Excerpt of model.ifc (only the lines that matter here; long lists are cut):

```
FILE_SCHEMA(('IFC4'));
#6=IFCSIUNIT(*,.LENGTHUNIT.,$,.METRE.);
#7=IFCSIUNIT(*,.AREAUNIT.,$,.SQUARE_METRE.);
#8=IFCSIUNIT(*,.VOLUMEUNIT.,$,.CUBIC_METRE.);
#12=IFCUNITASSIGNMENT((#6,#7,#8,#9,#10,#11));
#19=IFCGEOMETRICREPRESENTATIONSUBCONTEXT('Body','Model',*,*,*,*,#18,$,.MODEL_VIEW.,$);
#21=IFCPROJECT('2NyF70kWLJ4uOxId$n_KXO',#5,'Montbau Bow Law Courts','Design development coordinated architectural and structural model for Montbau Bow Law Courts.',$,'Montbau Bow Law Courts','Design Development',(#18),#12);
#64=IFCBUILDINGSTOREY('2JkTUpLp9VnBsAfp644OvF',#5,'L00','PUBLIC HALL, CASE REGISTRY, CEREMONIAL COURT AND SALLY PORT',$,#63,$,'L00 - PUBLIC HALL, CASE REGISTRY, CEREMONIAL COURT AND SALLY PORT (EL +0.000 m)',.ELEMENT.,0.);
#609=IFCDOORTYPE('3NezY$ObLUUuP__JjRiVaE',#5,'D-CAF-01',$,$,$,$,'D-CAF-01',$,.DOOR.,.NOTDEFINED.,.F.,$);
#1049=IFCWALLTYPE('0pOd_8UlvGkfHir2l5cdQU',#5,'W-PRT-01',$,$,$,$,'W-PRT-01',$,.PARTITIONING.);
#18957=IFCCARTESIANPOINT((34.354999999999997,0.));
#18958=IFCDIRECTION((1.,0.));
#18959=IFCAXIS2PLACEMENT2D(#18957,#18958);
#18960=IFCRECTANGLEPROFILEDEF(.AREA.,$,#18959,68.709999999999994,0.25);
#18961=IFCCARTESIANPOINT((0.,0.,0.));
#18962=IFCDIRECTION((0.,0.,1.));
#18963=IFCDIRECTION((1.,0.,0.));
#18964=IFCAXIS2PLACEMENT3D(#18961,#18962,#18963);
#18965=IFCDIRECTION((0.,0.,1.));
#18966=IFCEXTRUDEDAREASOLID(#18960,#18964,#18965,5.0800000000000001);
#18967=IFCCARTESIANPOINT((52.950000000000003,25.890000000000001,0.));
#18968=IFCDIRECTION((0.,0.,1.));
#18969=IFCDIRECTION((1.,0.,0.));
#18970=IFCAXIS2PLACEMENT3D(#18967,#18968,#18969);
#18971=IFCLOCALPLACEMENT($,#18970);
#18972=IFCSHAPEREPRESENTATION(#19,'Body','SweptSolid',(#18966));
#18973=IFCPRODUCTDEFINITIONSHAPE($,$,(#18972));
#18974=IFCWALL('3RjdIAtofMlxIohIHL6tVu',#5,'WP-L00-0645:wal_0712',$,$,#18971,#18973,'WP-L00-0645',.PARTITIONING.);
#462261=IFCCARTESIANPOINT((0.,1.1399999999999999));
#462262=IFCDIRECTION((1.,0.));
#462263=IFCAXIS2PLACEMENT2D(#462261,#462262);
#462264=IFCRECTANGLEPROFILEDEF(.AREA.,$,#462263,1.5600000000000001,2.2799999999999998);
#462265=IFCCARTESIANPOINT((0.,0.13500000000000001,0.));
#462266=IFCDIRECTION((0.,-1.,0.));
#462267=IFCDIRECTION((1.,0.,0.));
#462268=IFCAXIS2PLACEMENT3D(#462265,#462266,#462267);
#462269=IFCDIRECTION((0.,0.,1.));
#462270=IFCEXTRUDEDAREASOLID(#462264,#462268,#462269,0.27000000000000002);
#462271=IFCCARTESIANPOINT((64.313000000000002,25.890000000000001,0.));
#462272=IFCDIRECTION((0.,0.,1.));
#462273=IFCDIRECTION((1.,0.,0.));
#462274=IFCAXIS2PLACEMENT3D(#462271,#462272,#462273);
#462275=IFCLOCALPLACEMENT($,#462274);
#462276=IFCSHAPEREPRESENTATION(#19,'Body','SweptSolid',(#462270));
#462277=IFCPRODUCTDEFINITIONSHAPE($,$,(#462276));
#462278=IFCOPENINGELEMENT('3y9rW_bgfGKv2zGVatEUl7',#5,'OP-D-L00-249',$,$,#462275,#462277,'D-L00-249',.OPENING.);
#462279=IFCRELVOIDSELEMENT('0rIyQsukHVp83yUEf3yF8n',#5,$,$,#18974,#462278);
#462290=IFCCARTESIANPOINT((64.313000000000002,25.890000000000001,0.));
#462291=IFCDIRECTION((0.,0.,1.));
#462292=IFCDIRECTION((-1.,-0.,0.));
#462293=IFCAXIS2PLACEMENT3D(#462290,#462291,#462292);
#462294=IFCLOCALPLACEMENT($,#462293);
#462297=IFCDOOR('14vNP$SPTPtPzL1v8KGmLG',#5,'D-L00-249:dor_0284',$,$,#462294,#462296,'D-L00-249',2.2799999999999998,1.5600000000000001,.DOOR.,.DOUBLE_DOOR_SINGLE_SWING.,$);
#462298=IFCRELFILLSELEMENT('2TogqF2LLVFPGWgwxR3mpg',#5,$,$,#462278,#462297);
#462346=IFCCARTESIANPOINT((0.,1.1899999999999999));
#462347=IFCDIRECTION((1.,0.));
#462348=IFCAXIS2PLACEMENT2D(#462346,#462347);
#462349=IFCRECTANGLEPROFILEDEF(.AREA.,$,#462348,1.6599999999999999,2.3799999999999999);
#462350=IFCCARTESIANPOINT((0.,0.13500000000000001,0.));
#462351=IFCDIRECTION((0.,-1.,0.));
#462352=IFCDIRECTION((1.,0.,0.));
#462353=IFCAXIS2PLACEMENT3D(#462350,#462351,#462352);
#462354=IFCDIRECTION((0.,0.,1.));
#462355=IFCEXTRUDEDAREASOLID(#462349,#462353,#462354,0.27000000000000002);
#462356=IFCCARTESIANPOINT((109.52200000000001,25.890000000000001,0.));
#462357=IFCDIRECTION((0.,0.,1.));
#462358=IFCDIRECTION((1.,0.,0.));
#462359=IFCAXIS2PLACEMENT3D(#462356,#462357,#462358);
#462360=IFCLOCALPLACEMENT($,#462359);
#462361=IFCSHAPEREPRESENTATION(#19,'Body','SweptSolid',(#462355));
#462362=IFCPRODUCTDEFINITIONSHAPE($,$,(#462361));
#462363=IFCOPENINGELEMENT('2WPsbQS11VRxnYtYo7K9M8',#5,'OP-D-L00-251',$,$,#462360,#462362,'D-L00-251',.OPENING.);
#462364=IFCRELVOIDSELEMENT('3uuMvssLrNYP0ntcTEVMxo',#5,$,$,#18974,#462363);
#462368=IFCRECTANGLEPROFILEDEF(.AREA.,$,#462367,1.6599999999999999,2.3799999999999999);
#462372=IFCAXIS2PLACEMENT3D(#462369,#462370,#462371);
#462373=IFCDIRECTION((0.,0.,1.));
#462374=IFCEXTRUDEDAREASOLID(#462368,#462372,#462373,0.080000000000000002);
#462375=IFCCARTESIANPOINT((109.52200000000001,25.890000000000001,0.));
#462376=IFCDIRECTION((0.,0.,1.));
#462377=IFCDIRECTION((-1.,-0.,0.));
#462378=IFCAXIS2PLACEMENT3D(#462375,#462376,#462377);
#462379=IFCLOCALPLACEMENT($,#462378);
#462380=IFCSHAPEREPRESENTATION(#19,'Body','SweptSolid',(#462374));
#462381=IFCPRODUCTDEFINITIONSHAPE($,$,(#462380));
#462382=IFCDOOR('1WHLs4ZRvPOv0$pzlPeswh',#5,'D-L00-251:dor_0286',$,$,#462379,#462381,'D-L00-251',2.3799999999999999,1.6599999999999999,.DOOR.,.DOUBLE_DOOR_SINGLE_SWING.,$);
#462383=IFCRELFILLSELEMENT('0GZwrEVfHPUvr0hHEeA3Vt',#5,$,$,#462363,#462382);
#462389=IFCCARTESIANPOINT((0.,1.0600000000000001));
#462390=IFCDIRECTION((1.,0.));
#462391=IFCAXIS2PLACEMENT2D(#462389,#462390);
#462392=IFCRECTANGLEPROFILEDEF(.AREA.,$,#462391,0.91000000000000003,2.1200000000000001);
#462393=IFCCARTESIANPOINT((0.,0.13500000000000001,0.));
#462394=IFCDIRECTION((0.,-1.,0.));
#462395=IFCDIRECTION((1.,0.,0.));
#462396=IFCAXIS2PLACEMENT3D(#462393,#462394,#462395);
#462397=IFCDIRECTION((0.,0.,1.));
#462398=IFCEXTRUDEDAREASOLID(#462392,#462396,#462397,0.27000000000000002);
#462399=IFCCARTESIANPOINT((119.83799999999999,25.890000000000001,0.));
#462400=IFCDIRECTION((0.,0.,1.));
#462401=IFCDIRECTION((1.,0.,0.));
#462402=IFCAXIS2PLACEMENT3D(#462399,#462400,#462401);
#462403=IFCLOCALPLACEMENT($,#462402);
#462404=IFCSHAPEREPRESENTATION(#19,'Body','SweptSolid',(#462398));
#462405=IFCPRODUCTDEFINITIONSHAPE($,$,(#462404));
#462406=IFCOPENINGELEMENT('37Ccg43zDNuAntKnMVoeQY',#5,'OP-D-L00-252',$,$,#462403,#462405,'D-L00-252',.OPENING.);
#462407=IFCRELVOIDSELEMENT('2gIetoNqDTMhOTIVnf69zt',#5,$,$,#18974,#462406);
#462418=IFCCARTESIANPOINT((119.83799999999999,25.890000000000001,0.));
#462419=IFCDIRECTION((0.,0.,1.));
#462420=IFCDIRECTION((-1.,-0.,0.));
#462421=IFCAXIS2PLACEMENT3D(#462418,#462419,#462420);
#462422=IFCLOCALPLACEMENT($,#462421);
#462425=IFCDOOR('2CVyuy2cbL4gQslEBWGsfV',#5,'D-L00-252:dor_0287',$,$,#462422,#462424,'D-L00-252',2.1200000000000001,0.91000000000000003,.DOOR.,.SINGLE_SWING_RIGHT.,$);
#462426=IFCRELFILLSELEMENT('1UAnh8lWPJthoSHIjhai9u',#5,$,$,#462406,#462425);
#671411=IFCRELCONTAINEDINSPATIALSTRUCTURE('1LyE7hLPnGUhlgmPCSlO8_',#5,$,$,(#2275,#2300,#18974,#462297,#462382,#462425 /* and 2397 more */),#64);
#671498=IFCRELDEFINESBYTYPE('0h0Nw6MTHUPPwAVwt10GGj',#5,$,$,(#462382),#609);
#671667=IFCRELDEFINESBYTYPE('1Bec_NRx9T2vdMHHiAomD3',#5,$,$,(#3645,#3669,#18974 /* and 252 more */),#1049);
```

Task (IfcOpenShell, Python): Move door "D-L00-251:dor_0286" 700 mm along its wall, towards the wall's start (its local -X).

```python
import ifcopenshell
import ifcopenshell.api.geometry
import ifcopenshell.util.placement
import ifcopenshell.util.unit

model = ifcopenshell.open("model.ifc")
unit_scale = ifcopenshell.util.unit.calculate_unit_scale(model)

door = model.by_guid("1WHLs4ZRvPOv0$pzlPeswh")
opening = door.FillsVoids[0].RelatingOpeningElement
wall = opening.VoidsElements[0].RelatingBuildingElement

wall_matrix = ifcopenshell.util.placement.get_local_placement(wall.ObjectPlacement)
shift = wall_matrix[:3, 0] * -0.7 / unit_scale
before = ifcopenshell.util.placement.get_local_placement(door.ObjectPlacement)[:3, 3].copy()

# The door is not placed relative to its opening, so move both.
for product in (opening, door):
    matrix = ifcopenshell.util.placement.get_local_placement(product.ObjectPlacement)
    matrix[:3, 3] += shift
    ifcopenshell.api.geometry.edit_object_placement(model, product=product, matrix=matrix, is_si=False)

after = ifcopenshell.util.placement.get_local_placement(door.ObjectPlacement)[:3, 3]
print("door moved by", (after - before).round(3) + 0.0)

model.write("model_v2.ifc")
```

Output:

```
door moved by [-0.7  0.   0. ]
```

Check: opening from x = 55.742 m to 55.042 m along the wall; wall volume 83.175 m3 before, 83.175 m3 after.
